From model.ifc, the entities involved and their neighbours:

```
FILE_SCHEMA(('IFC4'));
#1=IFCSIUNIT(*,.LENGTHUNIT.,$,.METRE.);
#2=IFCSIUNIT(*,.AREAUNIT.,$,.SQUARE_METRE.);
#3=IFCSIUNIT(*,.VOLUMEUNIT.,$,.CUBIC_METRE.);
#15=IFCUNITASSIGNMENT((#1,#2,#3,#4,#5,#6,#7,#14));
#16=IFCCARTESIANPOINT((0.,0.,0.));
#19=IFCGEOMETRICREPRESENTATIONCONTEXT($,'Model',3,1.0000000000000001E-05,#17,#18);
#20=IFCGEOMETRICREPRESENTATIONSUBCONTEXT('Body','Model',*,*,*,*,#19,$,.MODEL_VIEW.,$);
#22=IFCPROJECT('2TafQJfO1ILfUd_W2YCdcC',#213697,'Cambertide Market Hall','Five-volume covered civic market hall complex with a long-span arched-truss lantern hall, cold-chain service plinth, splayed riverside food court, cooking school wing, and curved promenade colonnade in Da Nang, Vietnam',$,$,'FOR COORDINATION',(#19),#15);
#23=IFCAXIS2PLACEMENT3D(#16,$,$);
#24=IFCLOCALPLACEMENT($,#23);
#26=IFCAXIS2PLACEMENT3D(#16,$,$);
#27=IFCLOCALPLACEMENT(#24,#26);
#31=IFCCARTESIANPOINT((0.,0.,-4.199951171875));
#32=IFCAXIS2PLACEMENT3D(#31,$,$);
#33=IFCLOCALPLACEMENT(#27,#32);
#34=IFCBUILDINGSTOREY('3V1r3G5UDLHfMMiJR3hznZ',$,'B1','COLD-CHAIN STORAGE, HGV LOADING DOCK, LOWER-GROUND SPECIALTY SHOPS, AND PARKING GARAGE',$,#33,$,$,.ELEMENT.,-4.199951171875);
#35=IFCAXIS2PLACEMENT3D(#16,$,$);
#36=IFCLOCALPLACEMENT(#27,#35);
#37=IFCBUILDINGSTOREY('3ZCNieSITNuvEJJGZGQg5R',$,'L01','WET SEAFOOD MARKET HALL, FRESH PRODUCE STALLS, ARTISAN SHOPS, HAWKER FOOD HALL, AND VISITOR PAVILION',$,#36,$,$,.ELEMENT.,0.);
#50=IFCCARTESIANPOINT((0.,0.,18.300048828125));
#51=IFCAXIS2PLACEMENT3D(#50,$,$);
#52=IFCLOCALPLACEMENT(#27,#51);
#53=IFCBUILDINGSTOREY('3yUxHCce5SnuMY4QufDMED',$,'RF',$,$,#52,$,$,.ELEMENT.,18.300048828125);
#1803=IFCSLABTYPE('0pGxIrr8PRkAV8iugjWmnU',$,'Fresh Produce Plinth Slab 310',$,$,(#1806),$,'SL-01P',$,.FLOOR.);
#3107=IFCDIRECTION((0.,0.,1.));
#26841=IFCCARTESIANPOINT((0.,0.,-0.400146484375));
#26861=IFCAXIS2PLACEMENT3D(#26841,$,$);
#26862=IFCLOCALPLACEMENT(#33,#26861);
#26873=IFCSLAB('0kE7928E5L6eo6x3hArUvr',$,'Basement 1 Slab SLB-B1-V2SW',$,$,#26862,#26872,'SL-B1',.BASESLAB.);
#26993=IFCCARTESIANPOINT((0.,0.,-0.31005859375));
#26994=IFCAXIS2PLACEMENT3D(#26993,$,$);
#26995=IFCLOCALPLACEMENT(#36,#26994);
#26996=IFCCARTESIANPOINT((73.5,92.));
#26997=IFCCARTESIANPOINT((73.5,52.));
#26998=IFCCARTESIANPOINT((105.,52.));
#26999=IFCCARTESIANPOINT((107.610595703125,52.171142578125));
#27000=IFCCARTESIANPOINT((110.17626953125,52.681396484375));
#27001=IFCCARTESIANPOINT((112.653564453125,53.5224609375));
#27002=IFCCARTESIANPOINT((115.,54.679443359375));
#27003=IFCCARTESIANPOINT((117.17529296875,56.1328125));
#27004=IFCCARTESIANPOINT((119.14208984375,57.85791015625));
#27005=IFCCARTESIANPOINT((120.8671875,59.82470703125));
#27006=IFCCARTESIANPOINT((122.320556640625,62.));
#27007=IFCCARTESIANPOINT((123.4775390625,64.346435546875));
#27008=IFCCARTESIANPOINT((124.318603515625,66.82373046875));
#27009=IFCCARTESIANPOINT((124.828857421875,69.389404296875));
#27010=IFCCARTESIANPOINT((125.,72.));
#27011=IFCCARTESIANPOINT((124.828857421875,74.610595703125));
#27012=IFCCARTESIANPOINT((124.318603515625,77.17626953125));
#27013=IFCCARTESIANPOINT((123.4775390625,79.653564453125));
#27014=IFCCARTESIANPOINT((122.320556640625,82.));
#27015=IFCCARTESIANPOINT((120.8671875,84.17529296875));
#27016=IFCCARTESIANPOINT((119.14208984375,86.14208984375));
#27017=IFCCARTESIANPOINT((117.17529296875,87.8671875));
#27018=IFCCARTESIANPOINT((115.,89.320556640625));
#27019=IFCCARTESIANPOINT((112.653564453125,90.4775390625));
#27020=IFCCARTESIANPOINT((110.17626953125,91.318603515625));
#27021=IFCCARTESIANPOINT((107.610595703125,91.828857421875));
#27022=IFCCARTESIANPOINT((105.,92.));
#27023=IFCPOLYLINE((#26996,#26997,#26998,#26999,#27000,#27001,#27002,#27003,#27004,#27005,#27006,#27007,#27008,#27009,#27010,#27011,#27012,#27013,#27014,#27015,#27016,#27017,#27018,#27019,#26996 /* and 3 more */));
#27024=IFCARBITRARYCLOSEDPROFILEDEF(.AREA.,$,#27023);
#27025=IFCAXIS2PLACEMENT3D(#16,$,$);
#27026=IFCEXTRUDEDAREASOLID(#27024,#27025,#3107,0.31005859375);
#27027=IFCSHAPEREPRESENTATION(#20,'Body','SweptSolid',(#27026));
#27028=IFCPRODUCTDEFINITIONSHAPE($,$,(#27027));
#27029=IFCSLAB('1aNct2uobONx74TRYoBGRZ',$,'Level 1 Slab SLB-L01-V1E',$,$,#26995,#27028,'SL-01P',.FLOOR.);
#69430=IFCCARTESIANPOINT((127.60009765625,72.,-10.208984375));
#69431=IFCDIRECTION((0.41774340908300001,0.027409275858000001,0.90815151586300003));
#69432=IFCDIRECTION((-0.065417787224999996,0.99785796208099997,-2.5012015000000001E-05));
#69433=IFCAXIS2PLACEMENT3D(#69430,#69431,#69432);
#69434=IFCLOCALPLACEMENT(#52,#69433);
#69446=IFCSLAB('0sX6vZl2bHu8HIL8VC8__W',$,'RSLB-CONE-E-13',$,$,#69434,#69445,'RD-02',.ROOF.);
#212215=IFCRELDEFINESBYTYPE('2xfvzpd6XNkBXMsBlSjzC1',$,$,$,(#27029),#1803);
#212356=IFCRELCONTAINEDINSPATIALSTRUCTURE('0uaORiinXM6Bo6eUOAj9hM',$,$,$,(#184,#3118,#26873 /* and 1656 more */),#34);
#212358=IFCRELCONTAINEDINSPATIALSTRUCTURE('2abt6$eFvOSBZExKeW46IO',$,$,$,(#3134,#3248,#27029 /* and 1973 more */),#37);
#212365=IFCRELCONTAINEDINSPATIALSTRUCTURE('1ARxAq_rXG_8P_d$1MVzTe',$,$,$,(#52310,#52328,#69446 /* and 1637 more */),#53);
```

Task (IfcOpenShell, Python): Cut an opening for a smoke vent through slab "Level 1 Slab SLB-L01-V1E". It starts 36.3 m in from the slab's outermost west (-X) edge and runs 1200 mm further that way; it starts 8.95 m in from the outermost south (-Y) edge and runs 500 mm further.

```python
import numpy as np
import ifcopenshell
import ifcopenshell.api.feature
import ifcopenshell.api.geometry
import ifcopenshell.api.root
import ifcopenshell.geom
import ifcopenshell.util.placement
import ifcopenshell.util.representation
import ifcopenshell.util.shape
import ifcopenshell.util.unit

model = ifcopenshell.open("model.ifc")
unit_scale = ifcopenshell.util.unit.calculate_unit_scale(model)
settings = ifcopenshell.geom.settings()


def volume(element):
    """Net volume in cubic metres, openings subtracted."""
    shape = ifcopenshell.geom.create_shape(settings, element)
    return ifcopenshell.util.shape.get_volume(shape.geometry)


slab = model.by_guid("1aNct2uobONx74TRYoBGRZ")
before = volume(slab)

# Extent in the slab's own axes, in metres. The edges named are its -X and -Y sides.
slab_shape = ifcopenshell.geom.create_shape(settings, slab)
vertices = ifcopenshell.util.shape.get_vertices(slab_shape.geometry)
x_min, y_min, bottom = vertices.min(axis=0)
top = vertices[:, 2].max()

opening = ifcopenshell.api.root.create_entity(model, ifc_class="IfcOpeningElement", name="Smoke vent opening", predefined_type="OPENING")
context = ifcopenshell.util.representation.get_context(model, "Model", "Body", "MODEL_VIEW")
width, depth = 1.2, 0.5
outline = [(0.0, 0.0), (width, 0.0), (width, depth), (0.0, depth), (0.0, 0.0)]
# Overshoot both faces by 50 mm so the cut is clean.
shape = ifcopenshell.api.geometry.add_slab_representation(
    model, context=context, depth=top - bottom + 0.1, polyline=outline
)
ifcopenshell.api.geometry.assign_representation(model, product=opening, representation=shape)

matrix = ifcopenshell.util.placement.get_local_placement(slab.ObjectPlacement)
matrix[:, 3] = matrix @ np.append(np.array([x_min + 36.3, y_min + 8.95, bottom - 0.05]) / unit_scale, 1.0)
ifcopenshell.api.geometry.edit_object_placement(model, product=opening, matrix=matrix, is_si=False)
ifcopenshell.api.feature.add_feature(model, feature=opening, element=slab)

after = volume(slab)

print(f"slab volume {before:.3f} -> {after:.3f} m3")

model.write("model_v2.ifc")
```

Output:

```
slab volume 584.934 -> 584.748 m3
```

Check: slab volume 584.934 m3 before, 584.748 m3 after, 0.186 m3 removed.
